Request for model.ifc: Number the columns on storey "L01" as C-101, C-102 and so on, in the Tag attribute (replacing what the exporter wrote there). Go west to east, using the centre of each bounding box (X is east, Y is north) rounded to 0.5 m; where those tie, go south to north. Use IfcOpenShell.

First a look at what the model holds.

```python
import ifcopenshell
import ifcopenshell.util.element
import ifcopenshell.util.placement

model = ifcopenshell.open("model.ifc")
print(model.schema)
storey = next(s for s in model.by_type("IfcBuildingStorey") if s.Name == "L01")
columns = [e for e in ifcopenshell.util.element.get_decomposition(storey) if e.is_a("IfcColumn")]
for e in sorted(columns, key=lambda e: e.id()):
    origin = ifcopenshell.util.placement.get_local_placement(e.ObjectPlacement)[:3, 3]
    print(e.id(), e.Tag, e.Name, origin.round(2) + 0.0, sep=" | ")
```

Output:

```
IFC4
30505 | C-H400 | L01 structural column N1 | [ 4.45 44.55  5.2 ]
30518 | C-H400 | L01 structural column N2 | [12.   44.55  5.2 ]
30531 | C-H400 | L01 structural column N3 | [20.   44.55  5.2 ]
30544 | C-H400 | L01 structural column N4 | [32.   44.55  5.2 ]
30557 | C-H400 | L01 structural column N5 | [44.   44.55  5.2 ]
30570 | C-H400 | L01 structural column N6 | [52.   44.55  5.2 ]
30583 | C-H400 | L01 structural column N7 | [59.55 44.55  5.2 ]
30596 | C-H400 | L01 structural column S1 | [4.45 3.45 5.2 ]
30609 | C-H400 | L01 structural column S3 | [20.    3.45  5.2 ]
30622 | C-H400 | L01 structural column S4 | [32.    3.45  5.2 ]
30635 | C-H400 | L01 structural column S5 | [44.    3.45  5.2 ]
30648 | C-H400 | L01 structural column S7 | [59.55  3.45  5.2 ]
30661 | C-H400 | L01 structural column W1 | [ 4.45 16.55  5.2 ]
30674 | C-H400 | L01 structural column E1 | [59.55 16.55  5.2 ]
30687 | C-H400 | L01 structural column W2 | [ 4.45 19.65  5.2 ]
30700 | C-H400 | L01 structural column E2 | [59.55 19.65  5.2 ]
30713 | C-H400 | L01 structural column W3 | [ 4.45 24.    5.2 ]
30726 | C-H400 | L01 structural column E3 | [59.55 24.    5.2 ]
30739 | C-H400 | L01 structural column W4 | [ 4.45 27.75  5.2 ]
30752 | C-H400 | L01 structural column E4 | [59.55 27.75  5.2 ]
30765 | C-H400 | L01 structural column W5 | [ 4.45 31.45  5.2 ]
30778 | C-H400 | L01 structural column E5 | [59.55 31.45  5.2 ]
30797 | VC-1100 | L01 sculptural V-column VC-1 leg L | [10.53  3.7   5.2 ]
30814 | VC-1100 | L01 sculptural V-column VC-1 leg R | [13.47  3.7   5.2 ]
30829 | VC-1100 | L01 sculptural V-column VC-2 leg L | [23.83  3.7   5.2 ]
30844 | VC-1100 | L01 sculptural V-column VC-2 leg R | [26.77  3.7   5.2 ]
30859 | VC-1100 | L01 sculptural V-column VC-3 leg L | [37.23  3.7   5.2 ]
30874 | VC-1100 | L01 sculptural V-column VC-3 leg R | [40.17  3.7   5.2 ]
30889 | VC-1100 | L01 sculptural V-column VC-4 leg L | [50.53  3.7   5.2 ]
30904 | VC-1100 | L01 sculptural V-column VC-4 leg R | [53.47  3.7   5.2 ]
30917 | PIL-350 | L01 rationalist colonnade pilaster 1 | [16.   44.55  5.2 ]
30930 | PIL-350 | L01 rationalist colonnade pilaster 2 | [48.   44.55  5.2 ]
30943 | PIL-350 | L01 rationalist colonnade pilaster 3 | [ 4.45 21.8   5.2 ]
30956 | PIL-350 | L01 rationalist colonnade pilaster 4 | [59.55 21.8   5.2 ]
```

```python
import ifcopenshell
import ifcopenshell.geom
import ifcopenshell.util.element
import ifcopenshell.util.shape

model = ifcopenshell.open("model.ifc")
settings = ifcopenshell.geom.settings()
settings.set("use-world-coords", True)


def centre(element):
    shape = ifcopenshell.geom.create_shape(settings, element)
    return ifcopenshell.util.shape.get_bbox_centroid(shape.geometry)


storey = next(s for s in model.by_type("IfcBuildingStorey") if s.Name == "L01")
columns = [e for e in ifcopenshell.util.element.get_decomposition(storey) if e.is_a("IfcColumn")]

# Insertion points can sit at a corner or the storey origin, so sort by the geometry (in metres).
centres = {e: centre(e) for e in columns}
columns.sort(key=lambda e: (round(centres[e][0] / 0.5), centres[e][1]))

for i, e in enumerate(columns, start=1):
    number = f"C-1{i:02d}"
    e.Tag = number
    print(e.id(), number)

model.write("model_rev.ifc")
```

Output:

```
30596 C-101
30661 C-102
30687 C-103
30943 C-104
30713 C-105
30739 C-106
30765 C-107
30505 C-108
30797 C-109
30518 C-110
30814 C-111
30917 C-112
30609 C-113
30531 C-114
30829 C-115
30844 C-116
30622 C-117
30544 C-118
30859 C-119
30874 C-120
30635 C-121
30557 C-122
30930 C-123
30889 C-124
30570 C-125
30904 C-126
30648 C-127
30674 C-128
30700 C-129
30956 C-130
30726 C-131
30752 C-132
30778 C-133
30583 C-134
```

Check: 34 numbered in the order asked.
